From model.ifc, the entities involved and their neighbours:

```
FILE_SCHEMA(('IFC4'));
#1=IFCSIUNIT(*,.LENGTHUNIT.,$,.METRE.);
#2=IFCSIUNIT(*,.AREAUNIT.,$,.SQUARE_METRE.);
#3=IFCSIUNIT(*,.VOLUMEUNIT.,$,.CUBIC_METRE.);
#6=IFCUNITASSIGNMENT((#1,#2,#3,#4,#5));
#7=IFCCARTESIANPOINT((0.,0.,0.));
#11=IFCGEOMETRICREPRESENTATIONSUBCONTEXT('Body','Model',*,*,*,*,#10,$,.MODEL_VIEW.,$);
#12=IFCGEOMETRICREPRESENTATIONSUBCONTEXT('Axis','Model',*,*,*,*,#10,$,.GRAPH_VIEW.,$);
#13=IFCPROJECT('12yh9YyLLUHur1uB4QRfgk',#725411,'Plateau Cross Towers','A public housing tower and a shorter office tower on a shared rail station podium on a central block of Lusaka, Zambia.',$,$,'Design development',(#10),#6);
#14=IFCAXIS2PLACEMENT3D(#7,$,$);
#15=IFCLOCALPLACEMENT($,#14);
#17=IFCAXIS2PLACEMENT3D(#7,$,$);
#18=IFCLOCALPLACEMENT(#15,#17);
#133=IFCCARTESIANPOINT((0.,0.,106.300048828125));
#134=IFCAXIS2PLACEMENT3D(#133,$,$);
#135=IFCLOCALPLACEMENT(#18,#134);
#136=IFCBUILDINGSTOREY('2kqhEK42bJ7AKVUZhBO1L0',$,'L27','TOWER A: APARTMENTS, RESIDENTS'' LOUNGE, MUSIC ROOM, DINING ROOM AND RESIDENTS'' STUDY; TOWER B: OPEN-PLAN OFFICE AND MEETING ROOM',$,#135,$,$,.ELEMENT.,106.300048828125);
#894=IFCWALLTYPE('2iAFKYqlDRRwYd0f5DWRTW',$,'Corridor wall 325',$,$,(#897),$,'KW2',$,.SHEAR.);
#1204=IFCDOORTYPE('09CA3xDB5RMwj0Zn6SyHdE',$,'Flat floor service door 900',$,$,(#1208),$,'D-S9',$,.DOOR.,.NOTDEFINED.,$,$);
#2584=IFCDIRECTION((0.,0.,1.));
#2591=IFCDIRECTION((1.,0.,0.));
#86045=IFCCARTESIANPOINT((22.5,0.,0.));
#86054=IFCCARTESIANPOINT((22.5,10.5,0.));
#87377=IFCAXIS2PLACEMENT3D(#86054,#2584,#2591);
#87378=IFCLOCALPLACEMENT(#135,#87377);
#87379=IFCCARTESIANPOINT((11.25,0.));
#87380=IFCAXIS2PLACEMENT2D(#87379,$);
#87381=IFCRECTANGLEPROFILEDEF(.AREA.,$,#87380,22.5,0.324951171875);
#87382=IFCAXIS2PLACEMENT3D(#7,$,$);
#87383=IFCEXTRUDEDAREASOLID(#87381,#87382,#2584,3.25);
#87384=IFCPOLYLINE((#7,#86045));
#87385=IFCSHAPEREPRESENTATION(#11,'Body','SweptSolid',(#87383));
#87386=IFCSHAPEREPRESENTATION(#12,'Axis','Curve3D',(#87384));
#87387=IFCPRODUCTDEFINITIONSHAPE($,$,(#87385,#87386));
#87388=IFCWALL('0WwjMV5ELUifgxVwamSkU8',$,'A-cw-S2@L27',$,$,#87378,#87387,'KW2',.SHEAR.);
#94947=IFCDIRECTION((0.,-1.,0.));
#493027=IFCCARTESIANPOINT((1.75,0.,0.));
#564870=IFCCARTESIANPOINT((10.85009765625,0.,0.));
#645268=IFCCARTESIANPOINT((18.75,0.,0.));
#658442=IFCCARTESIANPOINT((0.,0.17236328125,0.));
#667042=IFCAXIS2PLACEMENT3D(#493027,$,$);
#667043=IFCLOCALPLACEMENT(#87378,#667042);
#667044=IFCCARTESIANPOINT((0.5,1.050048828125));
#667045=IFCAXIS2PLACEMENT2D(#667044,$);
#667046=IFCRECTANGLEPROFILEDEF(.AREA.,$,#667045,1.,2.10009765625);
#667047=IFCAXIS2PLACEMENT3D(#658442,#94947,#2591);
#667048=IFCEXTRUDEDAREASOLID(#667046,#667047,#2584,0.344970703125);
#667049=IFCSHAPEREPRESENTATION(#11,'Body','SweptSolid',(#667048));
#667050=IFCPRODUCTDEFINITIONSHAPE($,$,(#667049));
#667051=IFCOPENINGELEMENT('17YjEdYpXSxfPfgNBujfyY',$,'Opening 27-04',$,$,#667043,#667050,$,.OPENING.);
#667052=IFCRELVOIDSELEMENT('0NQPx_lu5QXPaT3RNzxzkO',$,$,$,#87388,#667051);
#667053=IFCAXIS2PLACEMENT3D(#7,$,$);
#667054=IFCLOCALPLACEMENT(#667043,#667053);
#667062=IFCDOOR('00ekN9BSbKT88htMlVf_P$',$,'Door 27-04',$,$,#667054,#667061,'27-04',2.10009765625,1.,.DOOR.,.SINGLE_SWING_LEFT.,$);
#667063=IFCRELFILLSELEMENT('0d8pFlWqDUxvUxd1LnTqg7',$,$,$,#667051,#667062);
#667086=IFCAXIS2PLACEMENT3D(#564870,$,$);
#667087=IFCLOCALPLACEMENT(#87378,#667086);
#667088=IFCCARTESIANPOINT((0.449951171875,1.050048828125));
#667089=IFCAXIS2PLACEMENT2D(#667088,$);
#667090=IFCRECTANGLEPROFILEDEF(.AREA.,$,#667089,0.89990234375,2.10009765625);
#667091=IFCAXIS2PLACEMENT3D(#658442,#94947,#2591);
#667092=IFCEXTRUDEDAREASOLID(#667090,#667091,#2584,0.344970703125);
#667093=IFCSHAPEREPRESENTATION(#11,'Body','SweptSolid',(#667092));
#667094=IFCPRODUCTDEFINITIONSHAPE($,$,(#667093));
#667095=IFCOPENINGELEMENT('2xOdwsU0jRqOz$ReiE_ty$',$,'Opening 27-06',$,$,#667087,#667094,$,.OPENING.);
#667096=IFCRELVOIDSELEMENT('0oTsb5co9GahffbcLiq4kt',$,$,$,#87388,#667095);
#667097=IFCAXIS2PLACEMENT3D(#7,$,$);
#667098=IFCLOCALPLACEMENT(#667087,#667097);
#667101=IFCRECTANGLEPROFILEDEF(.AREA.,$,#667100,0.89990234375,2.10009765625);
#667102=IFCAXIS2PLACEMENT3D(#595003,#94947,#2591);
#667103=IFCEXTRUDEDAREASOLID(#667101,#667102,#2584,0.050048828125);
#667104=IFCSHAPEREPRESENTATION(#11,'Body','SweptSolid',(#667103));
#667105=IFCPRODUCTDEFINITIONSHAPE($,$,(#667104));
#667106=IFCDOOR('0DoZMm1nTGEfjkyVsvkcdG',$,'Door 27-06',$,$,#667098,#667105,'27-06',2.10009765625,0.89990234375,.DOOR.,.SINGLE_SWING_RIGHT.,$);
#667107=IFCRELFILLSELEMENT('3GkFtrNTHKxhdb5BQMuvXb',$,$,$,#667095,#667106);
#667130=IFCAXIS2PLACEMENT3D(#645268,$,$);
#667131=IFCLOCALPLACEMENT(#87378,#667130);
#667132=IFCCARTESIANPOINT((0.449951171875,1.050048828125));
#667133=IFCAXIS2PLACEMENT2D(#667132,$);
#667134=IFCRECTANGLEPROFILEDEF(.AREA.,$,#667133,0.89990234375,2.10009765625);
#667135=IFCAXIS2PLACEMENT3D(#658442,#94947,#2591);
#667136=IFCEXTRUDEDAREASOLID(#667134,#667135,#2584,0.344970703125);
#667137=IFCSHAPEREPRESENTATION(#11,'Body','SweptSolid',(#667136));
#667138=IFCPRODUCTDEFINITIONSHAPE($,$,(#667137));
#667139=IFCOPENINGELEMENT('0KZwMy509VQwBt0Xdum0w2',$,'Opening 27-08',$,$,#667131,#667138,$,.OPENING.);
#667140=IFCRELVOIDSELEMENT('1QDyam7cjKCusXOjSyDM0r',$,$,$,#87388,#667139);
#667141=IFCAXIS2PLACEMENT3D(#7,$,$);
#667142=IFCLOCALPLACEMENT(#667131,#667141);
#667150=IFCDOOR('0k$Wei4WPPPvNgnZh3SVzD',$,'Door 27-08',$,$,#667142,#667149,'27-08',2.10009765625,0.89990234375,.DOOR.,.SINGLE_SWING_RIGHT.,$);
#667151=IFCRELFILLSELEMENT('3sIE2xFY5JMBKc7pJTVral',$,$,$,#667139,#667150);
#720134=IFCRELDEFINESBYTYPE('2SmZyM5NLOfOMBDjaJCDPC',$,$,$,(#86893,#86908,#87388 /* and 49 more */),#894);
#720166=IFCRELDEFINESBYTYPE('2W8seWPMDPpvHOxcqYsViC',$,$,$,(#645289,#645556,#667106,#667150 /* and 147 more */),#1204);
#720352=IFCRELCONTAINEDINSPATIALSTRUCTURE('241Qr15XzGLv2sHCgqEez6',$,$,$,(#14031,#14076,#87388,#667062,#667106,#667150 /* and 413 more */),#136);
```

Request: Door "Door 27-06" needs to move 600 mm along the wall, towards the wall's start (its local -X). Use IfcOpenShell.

```python
import ifcopenshell
import ifcopenshell.api.geometry
import ifcopenshell.util.placement

model = ifcopenshell.open("model.ifc")

door = model.by_guid("0DoZMm1nTGEfjkyVsvkcdG")
opening = door.FillsVoids[0].RelatingOpeningElement
wall = opening.VoidsElements[0].RelatingBuildingElement

wall_matrix = ifcopenshell.util.placement.get_local_placement(wall.ObjectPlacement)
shift = wall_matrix[:3, 0] * -0.6
before = ifcopenshell.util.placement.get_local_placement(door.ObjectPlacement)[:3, 3].copy()

# The door is placed relative to its opening, so it follows when the opening moves.
matrix = ifcopenshell.util.placement.get_local_placement(opening.ObjectPlacement)
matrix[:3, 3] += shift
ifcopenshell.api.geometry.edit_object_placement(
    model, product=opening, matrix=matrix, is_si=False, should_transform_children=True
)

after = ifcopenshell.util.placement.get_local_placement(door.ObjectPlacement)[:3, 3]
print("door moved by", (after - before).round(3) + 0.0)

model.write("model_edited.ifc")
```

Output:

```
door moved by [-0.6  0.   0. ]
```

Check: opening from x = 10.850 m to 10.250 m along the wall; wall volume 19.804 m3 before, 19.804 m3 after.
